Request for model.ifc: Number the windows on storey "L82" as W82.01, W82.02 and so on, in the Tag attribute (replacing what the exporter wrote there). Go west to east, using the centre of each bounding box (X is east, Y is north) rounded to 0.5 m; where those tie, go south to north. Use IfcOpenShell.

First a look at what the model holds.

```python
import ifcopenshell
import ifcopenshell.util.element
import ifcopenshell.util.placement

model = ifcopenshell.open("model.ifc")
print(model.schema)
storey = next(s for s in model.by_type("IfcBuildingStorey") if s.Name == "L82")
windows = [e for e in ifcopenshell.util.element.get_decomposition(storey) if e.is_a("IfcWindow")]
for e in sorted(windows, key=lambda e: e.id()):
    origin = ifcopenshell.util.placement.get_local_placement(e.ObjectPlacement)[:3, 3]
    print(e.id(), e.Tag, e.Name, origin.round(2) + 0.0, sep=" | ")
```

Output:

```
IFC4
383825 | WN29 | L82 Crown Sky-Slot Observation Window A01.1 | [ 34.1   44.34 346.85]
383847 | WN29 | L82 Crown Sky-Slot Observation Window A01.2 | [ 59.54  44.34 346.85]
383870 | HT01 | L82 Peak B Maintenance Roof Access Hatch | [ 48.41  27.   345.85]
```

```python
import ifcopenshell
import ifcopenshell.geom
import ifcopenshell.util.element
import ifcopenshell.util.shape

model = ifcopenshell.open("model.ifc")
settings = ifcopenshell.geom.settings()
settings.set("use-world-coords", True)


def centre(element):
    shape = ifcopenshell.geom.create_shape(settings, element)
    return ifcopenshell.util.shape.get_bbox_centroid(shape.geometry)


storey = next(s for s in model.by_type("IfcBuildingStorey") if s.Name == "L82")
windows = [e for e in ifcopenshell.util.element.get_decomposition(storey) if e.is_a("IfcWindow")]

# Insertion points can sit at a corner or the storey origin, so sort by the geometry (in metres).
centres = {e: centre(e) for e in windows}
windows.sort(key=lambda e: (round(centres[e][0] / 0.5), centres[e][1]))

for i, e in enumerate(windows, start=1):
    number = f"W82.{i:02d}"
    e.Tag = number
    print(e.id(), number)

model.write("model_rev.ifc")
```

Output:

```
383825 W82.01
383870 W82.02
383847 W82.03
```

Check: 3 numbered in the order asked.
